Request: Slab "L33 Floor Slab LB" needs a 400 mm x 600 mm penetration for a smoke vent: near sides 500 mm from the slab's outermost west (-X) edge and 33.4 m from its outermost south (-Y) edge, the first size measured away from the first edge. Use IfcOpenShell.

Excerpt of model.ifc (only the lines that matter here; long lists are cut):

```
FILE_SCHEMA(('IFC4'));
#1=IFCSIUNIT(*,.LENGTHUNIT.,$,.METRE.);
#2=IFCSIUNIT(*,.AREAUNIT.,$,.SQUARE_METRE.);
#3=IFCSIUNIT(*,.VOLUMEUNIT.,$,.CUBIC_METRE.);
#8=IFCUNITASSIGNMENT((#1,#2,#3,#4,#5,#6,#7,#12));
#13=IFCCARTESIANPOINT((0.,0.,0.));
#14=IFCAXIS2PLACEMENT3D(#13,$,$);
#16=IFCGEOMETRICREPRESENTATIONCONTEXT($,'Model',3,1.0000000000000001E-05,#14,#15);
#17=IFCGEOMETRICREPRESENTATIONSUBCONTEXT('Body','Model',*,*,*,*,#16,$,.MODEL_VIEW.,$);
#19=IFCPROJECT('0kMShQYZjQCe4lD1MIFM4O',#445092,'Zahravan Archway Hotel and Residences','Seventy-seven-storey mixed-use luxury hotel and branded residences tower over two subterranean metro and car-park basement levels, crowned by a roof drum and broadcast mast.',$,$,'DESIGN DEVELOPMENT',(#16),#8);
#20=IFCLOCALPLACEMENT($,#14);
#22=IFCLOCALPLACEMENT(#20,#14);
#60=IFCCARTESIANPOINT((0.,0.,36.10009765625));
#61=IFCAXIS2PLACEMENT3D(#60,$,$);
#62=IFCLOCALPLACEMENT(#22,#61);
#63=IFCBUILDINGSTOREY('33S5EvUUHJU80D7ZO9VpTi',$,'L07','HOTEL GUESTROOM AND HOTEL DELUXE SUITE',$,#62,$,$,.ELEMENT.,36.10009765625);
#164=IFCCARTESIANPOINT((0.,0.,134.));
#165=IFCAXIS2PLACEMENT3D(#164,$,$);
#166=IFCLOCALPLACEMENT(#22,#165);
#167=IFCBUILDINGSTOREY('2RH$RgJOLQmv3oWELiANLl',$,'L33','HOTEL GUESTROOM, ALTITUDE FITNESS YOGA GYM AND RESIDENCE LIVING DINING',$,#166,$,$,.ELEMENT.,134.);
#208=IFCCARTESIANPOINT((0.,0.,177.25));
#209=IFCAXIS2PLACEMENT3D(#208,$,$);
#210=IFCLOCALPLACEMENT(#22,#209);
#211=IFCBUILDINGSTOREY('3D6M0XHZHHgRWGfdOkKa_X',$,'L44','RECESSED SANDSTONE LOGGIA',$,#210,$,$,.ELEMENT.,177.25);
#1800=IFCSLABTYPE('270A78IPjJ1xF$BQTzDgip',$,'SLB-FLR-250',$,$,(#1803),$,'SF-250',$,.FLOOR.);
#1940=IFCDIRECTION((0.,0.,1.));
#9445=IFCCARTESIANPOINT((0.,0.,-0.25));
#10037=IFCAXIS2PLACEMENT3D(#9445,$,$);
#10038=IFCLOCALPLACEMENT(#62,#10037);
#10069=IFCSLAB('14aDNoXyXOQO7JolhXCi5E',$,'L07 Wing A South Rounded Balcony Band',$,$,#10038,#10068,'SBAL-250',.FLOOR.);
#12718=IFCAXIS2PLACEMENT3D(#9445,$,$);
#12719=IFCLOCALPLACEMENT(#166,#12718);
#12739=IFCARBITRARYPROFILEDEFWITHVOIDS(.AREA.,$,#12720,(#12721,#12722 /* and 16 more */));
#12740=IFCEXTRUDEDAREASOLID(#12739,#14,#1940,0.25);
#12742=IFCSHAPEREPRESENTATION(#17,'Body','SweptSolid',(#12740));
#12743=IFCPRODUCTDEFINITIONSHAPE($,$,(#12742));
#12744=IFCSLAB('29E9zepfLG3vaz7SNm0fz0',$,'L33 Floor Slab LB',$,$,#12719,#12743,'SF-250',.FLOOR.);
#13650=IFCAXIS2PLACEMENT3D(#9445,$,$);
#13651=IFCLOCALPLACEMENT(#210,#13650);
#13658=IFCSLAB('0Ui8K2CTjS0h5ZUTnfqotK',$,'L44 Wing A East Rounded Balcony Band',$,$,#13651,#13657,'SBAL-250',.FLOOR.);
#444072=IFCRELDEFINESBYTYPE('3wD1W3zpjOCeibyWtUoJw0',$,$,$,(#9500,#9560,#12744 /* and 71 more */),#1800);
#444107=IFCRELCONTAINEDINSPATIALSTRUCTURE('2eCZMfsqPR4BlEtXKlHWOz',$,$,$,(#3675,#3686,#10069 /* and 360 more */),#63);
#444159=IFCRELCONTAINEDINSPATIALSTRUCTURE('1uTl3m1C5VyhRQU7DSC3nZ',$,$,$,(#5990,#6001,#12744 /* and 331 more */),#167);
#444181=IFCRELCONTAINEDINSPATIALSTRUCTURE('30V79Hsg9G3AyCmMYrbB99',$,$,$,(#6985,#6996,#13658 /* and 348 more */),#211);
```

```python
import numpy as np
import ifcopenshell
import ifcopenshell.api.feature
import ifcopenshell.api.geometry
import ifcopenshell.api.root
import ifcopenshell.geom
import ifcopenshell.util.placement
import ifcopenshell.util.representation
import ifcopenshell.util.shape
import ifcopenshell.util.unit

model = ifcopenshell.open("model.ifc")
unit_scale = ifcopenshell.util.unit.calculate_unit_scale(model)
settings = ifcopenshell.geom.settings()


def volume(element):
    """Net volume in cubic metres, openings subtracted."""
    shape = ifcopenshell.geom.create_shape(settings, element)
    return ifcopenshell.util.shape.get_volume(shape.geometry)


slab = model.by_guid("29E9zepfLG3vaz7SNm0fz0")
before = volume(slab)

# Extent in the slab's own axes, in metres. The edges named are its -X and -Y sides.
slab_shape = ifcopenshell.geom.create_shape(settings, slab)
vertices = ifcopenshell.util.shape.get_vertices(slab_shape.geometry)
x_min, y_min, bottom = vertices.min(axis=0)
top = vertices[:, 2].max()

opening = ifcopenshell.api.root.create_entity(model, ifc_class="IfcOpeningElement", name="Smoke vent opening", predefined_type="OPENING")
context = ifcopenshell.util.representation.get_context(model, "Model", "Body", "MODEL_VIEW")
width, depth = 0.4, 0.6
outline = [(0.0, 0.0), (width, 0.0), (width, depth), (0.0, depth), (0.0, 0.0)]
# Overshoot both faces by 50 mm so the cut is clean.
shape = ifcopenshell.api.geometry.add_slab_representation(
    model, context=context, depth=top - bottom + 0.1, polyline=outline
)
ifcopenshell.api.geometry.assign_representation(model, product=opening, representation=shape)

matrix = ifcopenshell.util.placement.get_local_placement(slab.ObjectPlacement)
matrix[:, 3] = matrix @ np.append(np.array([x_min + 0.5, y_min + 33.4, bottom - 0.05]) / unit_scale, 1.0)
ifcopenshell.api.geometry.edit_object_placement(model, product=opening, matrix=matrix, is_si=False)
ifcopenshell.api.feature.add_feature(model, feature=opening, element=slab)

after = volume(slab)

print(f"slab volume {before:.3f} -> {after:.3f} m3")

model.write("model_rev.ifc")
```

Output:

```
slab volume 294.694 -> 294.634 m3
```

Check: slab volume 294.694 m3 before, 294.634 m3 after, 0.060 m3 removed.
